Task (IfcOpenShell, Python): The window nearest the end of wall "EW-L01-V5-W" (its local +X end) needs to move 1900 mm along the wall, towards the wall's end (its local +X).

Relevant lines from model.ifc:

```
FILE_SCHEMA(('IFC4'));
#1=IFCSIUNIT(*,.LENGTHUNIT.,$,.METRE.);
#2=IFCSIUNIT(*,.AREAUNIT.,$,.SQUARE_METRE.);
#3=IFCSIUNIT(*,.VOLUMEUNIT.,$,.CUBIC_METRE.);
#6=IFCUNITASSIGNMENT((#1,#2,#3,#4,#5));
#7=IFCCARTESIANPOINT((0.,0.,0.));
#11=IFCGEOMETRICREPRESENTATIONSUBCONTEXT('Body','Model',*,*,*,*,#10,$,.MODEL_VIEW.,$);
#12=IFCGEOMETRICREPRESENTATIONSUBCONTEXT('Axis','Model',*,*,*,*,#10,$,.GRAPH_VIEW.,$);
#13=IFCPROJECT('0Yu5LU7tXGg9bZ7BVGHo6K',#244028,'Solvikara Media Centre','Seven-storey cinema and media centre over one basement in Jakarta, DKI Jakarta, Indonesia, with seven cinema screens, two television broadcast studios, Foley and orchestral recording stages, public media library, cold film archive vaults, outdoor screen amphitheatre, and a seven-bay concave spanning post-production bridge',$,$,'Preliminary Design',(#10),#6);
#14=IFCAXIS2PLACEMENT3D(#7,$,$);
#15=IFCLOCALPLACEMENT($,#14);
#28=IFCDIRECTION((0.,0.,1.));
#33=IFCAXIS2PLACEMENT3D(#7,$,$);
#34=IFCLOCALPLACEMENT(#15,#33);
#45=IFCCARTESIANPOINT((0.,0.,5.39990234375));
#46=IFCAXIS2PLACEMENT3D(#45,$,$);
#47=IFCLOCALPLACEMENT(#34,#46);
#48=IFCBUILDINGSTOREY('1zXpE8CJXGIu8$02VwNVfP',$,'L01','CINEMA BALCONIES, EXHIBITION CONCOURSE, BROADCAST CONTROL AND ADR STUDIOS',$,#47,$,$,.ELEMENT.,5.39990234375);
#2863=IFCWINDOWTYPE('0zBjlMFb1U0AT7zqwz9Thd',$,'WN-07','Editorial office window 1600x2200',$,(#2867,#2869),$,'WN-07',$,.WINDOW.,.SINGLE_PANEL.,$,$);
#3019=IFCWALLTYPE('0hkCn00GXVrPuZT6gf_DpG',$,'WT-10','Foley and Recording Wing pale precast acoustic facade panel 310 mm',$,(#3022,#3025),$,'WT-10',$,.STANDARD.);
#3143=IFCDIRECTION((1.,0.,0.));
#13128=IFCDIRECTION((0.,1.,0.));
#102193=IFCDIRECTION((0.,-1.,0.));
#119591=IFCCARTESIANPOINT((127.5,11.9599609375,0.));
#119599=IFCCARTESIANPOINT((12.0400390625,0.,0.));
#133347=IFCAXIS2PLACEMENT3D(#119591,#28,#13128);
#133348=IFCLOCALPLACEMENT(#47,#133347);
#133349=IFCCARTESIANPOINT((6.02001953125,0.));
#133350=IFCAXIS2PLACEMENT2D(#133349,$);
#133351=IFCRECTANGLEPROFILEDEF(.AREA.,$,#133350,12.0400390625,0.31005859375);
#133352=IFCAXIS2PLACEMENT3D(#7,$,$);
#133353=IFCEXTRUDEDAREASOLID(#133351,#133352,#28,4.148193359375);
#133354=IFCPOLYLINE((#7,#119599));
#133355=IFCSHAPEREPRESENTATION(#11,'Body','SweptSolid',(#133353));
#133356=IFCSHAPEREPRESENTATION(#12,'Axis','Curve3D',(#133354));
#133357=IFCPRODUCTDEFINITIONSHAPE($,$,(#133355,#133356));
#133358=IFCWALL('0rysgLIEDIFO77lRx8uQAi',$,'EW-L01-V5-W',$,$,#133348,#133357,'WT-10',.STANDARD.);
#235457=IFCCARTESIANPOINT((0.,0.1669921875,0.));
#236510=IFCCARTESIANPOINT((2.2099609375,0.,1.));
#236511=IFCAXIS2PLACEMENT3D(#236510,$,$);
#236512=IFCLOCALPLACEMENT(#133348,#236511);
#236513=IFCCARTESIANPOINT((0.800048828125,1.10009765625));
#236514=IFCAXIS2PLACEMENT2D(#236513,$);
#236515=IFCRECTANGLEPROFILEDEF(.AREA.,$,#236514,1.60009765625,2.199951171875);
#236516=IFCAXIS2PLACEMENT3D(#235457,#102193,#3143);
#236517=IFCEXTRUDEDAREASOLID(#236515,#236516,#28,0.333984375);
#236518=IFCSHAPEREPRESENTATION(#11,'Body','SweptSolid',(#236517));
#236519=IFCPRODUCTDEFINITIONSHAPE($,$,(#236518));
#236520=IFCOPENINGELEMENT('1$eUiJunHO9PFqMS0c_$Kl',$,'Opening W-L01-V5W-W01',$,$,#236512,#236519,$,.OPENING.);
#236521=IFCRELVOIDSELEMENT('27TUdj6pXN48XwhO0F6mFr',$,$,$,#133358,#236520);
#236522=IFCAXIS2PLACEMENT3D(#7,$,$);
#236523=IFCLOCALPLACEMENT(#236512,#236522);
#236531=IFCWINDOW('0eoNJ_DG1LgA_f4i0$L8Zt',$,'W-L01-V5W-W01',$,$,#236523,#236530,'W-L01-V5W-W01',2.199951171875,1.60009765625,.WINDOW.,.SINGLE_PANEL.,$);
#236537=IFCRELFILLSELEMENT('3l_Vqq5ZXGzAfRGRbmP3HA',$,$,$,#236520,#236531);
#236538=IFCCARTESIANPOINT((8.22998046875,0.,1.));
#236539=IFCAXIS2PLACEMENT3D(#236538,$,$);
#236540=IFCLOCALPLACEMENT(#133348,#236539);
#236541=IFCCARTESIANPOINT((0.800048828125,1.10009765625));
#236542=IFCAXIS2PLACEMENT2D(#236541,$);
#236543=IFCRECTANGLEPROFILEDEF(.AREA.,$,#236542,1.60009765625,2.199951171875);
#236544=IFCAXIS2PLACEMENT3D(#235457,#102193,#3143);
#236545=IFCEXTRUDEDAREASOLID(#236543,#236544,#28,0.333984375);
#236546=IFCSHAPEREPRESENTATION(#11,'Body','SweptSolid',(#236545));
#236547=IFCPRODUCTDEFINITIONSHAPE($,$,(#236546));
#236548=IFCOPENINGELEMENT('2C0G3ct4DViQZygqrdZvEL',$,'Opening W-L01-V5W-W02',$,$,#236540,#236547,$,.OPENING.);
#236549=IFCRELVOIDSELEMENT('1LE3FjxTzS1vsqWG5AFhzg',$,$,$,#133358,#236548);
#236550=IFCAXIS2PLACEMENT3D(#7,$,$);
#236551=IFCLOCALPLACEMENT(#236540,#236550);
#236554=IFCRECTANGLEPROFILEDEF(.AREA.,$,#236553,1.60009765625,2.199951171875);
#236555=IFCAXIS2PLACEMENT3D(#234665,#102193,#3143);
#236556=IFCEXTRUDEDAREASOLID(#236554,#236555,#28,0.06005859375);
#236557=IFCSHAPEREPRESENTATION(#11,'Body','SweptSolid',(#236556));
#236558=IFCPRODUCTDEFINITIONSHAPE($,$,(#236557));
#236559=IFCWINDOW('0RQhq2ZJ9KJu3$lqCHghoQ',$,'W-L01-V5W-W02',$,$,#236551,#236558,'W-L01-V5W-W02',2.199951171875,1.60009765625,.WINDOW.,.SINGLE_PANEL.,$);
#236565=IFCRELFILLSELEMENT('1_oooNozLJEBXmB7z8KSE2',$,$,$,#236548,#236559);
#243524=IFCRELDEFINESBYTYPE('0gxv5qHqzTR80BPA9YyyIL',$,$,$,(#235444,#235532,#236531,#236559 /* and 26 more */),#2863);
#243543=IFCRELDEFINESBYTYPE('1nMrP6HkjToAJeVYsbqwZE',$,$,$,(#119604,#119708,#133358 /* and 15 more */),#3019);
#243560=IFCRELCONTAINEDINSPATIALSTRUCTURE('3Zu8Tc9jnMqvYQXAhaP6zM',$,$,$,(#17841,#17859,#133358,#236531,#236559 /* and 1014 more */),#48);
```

```python
import ifcopenshell
import ifcopenshell.api.geometry
import ifcopenshell.util.placement

model = ifcopenshell.open("model.ifc")

window = model.by_guid("0RQhq2ZJ9KJu3$lqCHghoQ")
opening = window.FillsVoids[0].RelatingOpeningElement
wall = opening.VoidsElements[0].RelatingBuildingElement

wall_matrix = ifcopenshell.util.placement.get_local_placement(wall.ObjectPlacement)
shift = wall_matrix[:3, 0] * 1.9
before = ifcopenshell.util.placement.get_local_placement(window.ObjectPlacement)[:3, 3].copy()

# The window is placed relative to its opening, so it follows when the opening moves.
matrix = ifcopenshell.util.placement.get_local_placement(opening.ObjectPlacement)
matrix[:3, 3] += shift
ifcopenshell.api.geometry.edit_object_placement(
    model, product=opening, matrix=matrix, is_si=False, should_transform_children=True
)

after = ifcopenshell.util.placement.get_local_placement(window.ObjectPlacement)[:3, 3]
print("window moved by", (after - before).round(3) + 0.0)

model.write("model_rev.ifc")
```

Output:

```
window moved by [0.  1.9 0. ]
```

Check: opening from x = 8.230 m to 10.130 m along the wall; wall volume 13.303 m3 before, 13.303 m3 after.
